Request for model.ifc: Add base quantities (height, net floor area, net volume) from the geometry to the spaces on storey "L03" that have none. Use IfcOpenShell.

First a look at what the model holds.

```python
import ifcopenshell
import ifcopenshell.util.element
import ifcopenshell.util.unit

model = ifcopenshell.open("model.ifc")
print(model.schema)
for unit_type in ("LENGTHUNIT", "AREAUNIT", "VOLUMEUNIT"):
    print(unit_type, ifcopenshell.util.unit.calculate_unit_scale(model, unit_type))
storey = next(s for s in model.by_type("IfcBuildingStorey") if s.Name == "L03")
spaces = [e for e in ifcopenshell.util.element.get_decomposition(storey) if e.is_a("IfcSpace")]
for e in sorted(spaces, key=lambda e: e.id()):
    print(e.id(), e.is_a(), e.Name, list(ifcopenshell.util.element.get_psets(e, qtos_only=True)), sep=" | ")
```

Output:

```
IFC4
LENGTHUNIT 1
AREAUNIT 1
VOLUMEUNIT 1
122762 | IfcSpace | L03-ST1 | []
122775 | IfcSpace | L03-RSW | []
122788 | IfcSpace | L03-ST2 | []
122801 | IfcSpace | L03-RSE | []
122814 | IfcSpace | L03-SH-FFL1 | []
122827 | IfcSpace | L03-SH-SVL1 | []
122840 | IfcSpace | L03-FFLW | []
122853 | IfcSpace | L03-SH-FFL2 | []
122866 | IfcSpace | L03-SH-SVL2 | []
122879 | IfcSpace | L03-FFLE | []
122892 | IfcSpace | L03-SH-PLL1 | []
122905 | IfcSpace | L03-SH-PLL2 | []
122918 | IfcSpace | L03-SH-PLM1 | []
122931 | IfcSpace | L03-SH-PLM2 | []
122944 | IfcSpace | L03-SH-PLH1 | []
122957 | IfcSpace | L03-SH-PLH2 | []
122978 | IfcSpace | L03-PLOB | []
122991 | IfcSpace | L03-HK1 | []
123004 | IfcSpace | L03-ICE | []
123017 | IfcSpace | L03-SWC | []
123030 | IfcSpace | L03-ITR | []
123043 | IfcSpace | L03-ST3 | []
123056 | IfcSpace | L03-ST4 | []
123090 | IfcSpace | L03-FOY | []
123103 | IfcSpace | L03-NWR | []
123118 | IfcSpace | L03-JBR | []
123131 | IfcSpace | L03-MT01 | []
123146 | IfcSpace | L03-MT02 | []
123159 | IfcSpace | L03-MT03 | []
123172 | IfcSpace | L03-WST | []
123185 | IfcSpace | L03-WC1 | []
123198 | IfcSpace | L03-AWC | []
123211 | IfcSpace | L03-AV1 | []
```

```python
import ifcopenshell
import ifcopenshell.api.pset
import ifcopenshell.geom
import ifcopenshell.util.element
import ifcopenshell.util.shape
import ifcopenshell.util.unit

model = ifcopenshell.open("model.ifc")
unit_scale = ifcopenshell.util.unit.calculate_unit_scale(model)
area_scale = ifcopenshell.util.unit.calculate_unit_scale(model, "AREAUNIT")
volume_scale = ifcopenshell.util.unit.calculate_unit_scale(model, "VOLUMEUNIT")
settings = ifcopenshell.geom.settings()

storey = next(s for s in model.by_type("IfcBuildingStorey") if s.Name == "L03")
spaces = [e for e in ifcopenshell.util.element.get_decomposition(storey) if e.is_a("IfcSpace")]

for e in sorted(spaces, key=lambda e: e.id()):
    if ifcopenshell.util.element.get_psets(e, qtos_only=True, should_inherit=False):
        continue
    # Geometry comes back in metres, in the element's own axes.
    shape = ifcopenshell.geom.create_shape(settings, e)
    values = {
        "Height": ifcopenshell.util.shape.get_z(shape.geometry) / unit_scale,
        "NetFloorArea": ifcopenshell.util.shape.get_footprint_area(shape.geometry) / area_scale,
        "NetVolume": ifcopenshell.util.shape.get_volume(shape.geometry) / volume_scale,
    }
    qto = ifcopenshell.api.pset.add_qto(model, product=e, name="Qto_SpaceBaseQuantities")
    ifcopenshell.api.pset.edit_qto(model, qto=qto, properties=values)
    print(e.id(), {k: round(v, 3) for k, v in values.items()})

model.write("model_rev.ifc")
```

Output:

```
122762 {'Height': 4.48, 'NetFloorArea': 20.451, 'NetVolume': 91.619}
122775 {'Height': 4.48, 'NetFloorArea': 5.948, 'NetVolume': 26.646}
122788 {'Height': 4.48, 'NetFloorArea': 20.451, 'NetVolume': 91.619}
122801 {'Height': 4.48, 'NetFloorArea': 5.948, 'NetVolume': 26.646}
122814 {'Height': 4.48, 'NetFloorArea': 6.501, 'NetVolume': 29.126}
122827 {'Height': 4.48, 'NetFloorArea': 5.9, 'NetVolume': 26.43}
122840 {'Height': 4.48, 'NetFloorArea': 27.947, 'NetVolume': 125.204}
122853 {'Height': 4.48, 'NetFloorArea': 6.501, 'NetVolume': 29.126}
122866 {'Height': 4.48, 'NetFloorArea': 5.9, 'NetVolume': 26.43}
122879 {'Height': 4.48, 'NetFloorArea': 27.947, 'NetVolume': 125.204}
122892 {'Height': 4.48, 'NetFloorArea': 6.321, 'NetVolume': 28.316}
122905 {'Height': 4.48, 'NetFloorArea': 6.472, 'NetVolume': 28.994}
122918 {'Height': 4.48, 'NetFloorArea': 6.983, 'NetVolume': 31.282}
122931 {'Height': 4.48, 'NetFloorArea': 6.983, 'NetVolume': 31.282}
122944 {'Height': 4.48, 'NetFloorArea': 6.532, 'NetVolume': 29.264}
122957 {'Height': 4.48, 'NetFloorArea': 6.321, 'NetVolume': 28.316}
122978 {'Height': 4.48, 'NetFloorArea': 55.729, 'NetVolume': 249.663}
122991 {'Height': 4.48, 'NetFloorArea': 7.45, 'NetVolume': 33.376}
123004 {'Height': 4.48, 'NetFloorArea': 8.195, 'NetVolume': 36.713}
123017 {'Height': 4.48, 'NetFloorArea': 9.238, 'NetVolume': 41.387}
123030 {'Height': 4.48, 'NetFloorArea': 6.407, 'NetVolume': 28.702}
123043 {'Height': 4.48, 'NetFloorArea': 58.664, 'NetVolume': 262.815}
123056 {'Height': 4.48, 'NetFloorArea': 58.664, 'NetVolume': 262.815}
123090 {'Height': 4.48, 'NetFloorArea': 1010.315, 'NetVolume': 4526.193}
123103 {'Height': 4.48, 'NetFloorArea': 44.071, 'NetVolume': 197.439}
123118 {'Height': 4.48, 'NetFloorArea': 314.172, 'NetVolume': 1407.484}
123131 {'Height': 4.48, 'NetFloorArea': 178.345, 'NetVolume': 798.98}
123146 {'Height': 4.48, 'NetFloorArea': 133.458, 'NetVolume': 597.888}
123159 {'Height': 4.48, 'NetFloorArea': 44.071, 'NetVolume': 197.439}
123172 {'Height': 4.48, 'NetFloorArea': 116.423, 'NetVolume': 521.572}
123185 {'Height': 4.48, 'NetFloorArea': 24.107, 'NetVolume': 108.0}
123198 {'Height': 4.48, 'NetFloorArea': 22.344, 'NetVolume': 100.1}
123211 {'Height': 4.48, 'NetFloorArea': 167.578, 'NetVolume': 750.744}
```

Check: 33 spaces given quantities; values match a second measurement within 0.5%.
